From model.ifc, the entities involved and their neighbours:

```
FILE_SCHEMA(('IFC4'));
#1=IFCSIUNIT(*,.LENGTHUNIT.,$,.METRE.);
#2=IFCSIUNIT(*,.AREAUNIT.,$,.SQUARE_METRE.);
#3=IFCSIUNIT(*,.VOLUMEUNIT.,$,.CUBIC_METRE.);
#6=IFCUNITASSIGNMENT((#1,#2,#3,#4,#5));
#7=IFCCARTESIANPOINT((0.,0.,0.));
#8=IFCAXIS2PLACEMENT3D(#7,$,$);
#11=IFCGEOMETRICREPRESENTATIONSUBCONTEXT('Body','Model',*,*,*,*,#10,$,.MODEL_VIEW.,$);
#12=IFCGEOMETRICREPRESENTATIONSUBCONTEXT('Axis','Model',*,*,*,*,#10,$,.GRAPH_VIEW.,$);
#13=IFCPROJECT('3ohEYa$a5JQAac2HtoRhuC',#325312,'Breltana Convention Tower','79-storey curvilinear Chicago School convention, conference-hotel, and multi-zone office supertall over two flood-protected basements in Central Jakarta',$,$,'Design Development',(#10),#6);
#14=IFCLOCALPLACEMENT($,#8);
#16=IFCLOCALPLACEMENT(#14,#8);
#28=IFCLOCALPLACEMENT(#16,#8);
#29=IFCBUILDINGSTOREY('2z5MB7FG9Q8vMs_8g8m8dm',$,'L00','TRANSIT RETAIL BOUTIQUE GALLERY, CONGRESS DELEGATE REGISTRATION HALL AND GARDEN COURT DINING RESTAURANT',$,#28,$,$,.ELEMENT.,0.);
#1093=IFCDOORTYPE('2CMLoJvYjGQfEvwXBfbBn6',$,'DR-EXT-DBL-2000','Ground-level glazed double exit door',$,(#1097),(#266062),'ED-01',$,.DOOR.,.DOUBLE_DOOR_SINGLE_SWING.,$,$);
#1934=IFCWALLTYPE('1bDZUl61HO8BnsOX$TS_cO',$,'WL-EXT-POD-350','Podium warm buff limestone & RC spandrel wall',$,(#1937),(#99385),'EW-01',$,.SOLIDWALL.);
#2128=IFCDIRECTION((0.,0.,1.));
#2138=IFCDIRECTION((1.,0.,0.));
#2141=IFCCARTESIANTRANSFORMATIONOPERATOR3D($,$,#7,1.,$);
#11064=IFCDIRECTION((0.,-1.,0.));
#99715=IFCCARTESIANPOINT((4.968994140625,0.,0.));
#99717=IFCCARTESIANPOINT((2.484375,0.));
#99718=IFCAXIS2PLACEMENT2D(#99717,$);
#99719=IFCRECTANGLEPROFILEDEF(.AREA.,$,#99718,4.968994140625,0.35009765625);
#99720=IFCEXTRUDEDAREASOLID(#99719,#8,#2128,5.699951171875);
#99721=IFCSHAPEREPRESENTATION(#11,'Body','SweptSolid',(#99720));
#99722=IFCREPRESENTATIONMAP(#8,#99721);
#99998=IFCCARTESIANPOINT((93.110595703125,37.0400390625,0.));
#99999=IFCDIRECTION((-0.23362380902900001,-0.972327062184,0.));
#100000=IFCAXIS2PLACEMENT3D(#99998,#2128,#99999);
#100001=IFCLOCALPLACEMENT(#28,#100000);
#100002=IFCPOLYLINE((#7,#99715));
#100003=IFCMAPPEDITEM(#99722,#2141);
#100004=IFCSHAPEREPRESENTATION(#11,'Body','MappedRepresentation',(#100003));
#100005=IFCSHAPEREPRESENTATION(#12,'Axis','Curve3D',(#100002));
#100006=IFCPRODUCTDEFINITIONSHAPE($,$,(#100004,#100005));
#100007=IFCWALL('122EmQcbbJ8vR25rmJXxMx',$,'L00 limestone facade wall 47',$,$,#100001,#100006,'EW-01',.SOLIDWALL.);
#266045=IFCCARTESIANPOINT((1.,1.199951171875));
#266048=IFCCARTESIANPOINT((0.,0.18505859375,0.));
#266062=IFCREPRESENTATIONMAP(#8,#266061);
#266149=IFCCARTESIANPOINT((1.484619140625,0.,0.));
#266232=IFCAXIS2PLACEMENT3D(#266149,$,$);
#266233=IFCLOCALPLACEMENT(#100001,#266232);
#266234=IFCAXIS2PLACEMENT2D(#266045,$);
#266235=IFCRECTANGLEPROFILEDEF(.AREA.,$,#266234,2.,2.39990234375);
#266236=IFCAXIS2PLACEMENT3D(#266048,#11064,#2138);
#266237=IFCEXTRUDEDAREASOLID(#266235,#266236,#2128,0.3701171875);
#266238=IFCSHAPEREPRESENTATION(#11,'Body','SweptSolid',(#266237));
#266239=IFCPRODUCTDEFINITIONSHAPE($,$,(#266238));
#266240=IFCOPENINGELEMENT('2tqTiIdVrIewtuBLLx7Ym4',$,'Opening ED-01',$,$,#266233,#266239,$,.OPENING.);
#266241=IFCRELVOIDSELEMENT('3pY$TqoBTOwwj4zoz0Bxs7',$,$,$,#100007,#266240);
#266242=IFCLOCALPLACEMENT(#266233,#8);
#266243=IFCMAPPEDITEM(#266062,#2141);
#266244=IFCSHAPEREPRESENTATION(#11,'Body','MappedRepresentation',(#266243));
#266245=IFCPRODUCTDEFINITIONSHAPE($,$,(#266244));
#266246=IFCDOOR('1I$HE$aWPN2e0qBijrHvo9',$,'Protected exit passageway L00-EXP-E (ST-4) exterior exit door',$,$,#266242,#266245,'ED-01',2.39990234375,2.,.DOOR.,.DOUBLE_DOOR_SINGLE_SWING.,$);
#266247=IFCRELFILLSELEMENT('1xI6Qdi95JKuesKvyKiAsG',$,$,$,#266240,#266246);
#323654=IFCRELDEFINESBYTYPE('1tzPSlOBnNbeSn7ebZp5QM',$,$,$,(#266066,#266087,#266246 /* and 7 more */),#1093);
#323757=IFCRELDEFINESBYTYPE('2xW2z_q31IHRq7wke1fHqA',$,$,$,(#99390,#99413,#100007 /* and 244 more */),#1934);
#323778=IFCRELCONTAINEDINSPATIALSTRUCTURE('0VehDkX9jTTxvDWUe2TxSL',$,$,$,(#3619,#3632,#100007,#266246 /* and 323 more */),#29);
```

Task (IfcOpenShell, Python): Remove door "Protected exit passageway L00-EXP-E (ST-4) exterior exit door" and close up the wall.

```python
import ifcopenshell
import ifcopenshell.api.feature
import ifcopenshell.api.root
import ifcopenshell.geom
import ifcopenshell.util.shape

model = ifcopenshell.open("model.ifc")
settings = ifcopenshell.geom.settings()


def volume(element):
    """Net volume in cubic metres, openings subtracted."""
    shape = ifcopenshell.geom.create_shape(settings, element)
    return ifcopenshell.util.shape.get_volume(shape.geometry)


door = model.by_id(266246)
opening = door.FillsVoids[0].RelatingOpeningElement
wall = opening.VoidsElements[0].RelatingBuildingElement
before = volume(wall)

ifcopenshell.api.root.remove_product(model, product=door)
ifcopenshell.api.feature.remove_feature(model, feature=opening)

after = volume(wall)

print(f"wall volume {before:.3f} -> {after:.3f} m3")

model.write("model_updated.ifc")
```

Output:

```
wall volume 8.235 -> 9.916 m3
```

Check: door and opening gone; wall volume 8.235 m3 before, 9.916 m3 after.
